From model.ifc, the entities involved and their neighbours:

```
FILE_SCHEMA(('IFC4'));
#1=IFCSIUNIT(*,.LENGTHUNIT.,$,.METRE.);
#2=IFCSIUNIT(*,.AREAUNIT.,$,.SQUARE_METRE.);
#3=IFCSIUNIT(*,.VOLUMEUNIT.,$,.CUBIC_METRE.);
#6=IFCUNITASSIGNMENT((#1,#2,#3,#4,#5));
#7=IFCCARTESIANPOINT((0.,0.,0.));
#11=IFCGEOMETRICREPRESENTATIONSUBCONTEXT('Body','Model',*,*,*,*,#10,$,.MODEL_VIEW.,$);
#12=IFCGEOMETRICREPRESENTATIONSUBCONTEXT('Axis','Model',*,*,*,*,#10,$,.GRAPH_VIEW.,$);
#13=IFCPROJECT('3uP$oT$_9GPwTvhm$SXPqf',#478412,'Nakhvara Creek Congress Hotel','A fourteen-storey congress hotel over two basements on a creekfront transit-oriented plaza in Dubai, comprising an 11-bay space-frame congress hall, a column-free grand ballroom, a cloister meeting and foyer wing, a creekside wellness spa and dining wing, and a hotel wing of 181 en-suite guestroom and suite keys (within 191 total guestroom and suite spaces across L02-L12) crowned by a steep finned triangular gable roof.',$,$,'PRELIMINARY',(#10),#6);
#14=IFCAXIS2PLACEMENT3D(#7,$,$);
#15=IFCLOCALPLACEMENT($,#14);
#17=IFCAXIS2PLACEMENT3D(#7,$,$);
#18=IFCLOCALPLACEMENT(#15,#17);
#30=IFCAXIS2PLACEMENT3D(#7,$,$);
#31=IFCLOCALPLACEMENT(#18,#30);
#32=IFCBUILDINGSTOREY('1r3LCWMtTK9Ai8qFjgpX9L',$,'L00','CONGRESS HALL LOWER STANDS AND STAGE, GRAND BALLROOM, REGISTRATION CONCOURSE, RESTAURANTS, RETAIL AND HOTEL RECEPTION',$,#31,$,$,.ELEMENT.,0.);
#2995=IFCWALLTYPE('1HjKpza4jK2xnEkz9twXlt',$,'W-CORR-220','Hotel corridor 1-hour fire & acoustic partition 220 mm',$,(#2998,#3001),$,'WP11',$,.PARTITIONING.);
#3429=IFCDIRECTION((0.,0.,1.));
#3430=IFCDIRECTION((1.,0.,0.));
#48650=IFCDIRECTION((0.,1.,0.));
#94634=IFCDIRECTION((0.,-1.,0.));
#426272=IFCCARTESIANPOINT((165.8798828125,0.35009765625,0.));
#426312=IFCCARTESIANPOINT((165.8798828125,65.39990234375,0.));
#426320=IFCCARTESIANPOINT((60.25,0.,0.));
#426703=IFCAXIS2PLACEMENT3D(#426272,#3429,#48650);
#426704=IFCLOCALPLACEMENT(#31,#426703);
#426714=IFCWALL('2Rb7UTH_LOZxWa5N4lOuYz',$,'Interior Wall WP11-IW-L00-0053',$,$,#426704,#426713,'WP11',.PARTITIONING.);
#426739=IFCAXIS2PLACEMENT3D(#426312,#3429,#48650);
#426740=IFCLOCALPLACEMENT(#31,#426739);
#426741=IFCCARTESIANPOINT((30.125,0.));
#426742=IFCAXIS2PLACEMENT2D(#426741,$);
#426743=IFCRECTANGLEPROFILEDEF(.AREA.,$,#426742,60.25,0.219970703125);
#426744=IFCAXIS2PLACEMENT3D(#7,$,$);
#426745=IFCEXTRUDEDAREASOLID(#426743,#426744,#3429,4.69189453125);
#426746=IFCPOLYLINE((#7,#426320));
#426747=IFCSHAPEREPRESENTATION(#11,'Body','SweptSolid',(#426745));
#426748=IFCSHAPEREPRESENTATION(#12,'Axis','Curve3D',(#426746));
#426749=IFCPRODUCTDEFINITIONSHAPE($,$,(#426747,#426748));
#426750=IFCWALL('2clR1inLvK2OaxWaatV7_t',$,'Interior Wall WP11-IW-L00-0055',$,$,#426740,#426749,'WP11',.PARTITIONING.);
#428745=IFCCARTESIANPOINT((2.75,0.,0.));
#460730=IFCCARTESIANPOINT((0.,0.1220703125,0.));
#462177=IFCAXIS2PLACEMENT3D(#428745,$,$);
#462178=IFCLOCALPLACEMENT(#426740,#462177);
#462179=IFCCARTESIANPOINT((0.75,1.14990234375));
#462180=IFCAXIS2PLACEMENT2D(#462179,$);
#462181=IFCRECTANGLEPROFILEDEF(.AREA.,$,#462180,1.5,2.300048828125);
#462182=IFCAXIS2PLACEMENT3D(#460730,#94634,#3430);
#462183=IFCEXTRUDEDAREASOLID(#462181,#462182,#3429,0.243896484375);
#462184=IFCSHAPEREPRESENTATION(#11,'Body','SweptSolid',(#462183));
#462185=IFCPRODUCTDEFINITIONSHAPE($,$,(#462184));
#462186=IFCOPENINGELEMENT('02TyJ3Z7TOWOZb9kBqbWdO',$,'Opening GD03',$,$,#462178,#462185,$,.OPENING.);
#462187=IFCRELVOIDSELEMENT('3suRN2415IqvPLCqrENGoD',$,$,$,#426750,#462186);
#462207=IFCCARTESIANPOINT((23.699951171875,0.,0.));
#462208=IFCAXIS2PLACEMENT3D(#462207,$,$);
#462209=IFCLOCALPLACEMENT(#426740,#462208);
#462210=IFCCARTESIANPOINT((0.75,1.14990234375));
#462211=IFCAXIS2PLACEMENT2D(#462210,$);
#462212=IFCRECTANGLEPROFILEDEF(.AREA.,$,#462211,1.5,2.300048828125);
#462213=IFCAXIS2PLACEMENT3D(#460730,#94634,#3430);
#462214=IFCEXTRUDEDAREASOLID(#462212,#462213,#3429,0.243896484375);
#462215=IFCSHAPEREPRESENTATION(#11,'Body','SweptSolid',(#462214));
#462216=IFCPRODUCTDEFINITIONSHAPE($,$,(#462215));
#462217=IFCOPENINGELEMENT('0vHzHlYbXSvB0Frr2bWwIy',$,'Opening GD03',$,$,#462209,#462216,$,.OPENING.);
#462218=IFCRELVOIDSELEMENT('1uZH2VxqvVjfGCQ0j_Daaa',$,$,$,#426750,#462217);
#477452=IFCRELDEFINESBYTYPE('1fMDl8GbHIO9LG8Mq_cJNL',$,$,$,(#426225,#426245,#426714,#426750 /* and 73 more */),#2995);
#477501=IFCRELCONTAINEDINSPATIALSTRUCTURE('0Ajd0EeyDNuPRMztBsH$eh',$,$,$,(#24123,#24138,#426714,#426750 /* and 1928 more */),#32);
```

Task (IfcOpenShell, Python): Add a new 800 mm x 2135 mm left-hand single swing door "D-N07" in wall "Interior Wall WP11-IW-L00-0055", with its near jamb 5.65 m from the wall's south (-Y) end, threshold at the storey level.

```python
import numpy as np
import ifcopenshell
import ifcopenshell.api.feature
import ifcopenshell.api.geometry
import ifcopenshell.api.root
import ifcopenshell.api.spatial
import ifcopenshell.geom
import ifcopenshell.util.element
import ifcopenshell.util.placement
import ifcopenshell.util.representation
import ifcopenshell.util.shape
import ifcopenshell.util.unit

model = ifcopenshell.open("model.ifc")
unit_scale = ifcopenshell.util.unit.calculate_unit_scale(model)
settings = ifcopenshell.geom.settings()


def volume(element):
    """Net volume in cubic metres, openings subtracted."""
    shape = ifcopenshell.geom.create_shape(settings, element)
    return ifcopenshell.util.shape.get_volume(shape.geometry)


wall = model.by_guid("2clR1inLvK2OaxWaatV7_t")
storey = ifcopenshell.util.element.get_container(wall, ifc_class="IfcBuildingStorey")
context = ifcopenshell.util.representation.get_context(model, "Model", "Body", "MODEL_VIEW")
before = volume(wall)

width, height, from_end, sill = 0.8, 2.135, 5.65, 0.0  # metres

# The wall runs along its own X axis, and the end named is its -X end.
wall_shape = ifcopenshell.geom.create_shape(settings, wall)
x, y, z = ifcopenshell.util.shape.get_vertices(wall_shape.geometry).T
start = x.min() + from_end
face, thickness = float(y.min()), float(y.max() - y.min())
wall_matrix = ifcopenshell.util.placement.get_local_placement(wall.ObjectPlacement)
level = ifcopenshell.util.placement.get_local_placement(storey.ObjectPlacement)[2, 3]


def in_wall(x, y):
    """Placement at x, y metres in the wall's axes, at sill height."""
    matrix = wall_matrix.copy()
    matrix[:, 3] = wall_matrix @ np.array([x / unit_scale, y / unit_scale, 0.0, 1.0])
    matrix[2, 3] = level + sill / unit_scale
    return matrix


# Opening: a box that overshoots both wall faces by 50 mm.
opening = ifcopenshell.api.root.create_entity(model, ifc_class="IfcOpeningElement", predefined_type="OPENING")
box = ifcopenshell.api.geometry.add_wall_representation(
    model, context=context, length=width, height=height, thickness=thickness + 0.1
)
ifcopenshell.api.geometry.assign_representation(model, product=opening, representation=box)
ifcopenshell.api.geometry.edit_object_placement(model, product=opening, matrix=in_wall(start, face - 0.05), is_si=False)
ifcopenshell.api.feature.add_feature(model, feature=opening, element=wall)

door = ifcopenshell.api.root.create_entity(model, ifc_class="IfcDoor", name="D-N07", predefined_type="DOOR")
door.OverallWidth, door.OverallHeight = width / unit_scale, height / unit_scale
door.OperationType = "SINGLE_SWING_LEFT"
body = ifcopenshell.api.geometry.add_door_representation(
    model,
    context=context,
    overall_width=door.OverallWidth,
    overall_height=door.OverallHeight,
    operation_type="SINGLE_SWING_LEFT",
    lining_properties={"LiningDepth": thickness / unit_scale, "ThresholdDepth": thickness / unit_scale},
)
ifcopenshell.api.geometry.assign_representation(model, product=door, representation=body)
ifcopenshell.api.spatial.assign_container(model, products=[door], relating_structure=storey)
ifcopenshell.api.feature.add_filling(model, opening=opening, element=door)

# The lining spans the wall, so the door starts at the wall face.
ifcopenshell.api.geometry.edit_object_placement(model, product=door, matrix=in_wall(start, face), is_si=False)

after = volume(wall)

print(f"wall volume {before:.3f} -> {after:.3f} m3")

model.write("model-out.ifc")
```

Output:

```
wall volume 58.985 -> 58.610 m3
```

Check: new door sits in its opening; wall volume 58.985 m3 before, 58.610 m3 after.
